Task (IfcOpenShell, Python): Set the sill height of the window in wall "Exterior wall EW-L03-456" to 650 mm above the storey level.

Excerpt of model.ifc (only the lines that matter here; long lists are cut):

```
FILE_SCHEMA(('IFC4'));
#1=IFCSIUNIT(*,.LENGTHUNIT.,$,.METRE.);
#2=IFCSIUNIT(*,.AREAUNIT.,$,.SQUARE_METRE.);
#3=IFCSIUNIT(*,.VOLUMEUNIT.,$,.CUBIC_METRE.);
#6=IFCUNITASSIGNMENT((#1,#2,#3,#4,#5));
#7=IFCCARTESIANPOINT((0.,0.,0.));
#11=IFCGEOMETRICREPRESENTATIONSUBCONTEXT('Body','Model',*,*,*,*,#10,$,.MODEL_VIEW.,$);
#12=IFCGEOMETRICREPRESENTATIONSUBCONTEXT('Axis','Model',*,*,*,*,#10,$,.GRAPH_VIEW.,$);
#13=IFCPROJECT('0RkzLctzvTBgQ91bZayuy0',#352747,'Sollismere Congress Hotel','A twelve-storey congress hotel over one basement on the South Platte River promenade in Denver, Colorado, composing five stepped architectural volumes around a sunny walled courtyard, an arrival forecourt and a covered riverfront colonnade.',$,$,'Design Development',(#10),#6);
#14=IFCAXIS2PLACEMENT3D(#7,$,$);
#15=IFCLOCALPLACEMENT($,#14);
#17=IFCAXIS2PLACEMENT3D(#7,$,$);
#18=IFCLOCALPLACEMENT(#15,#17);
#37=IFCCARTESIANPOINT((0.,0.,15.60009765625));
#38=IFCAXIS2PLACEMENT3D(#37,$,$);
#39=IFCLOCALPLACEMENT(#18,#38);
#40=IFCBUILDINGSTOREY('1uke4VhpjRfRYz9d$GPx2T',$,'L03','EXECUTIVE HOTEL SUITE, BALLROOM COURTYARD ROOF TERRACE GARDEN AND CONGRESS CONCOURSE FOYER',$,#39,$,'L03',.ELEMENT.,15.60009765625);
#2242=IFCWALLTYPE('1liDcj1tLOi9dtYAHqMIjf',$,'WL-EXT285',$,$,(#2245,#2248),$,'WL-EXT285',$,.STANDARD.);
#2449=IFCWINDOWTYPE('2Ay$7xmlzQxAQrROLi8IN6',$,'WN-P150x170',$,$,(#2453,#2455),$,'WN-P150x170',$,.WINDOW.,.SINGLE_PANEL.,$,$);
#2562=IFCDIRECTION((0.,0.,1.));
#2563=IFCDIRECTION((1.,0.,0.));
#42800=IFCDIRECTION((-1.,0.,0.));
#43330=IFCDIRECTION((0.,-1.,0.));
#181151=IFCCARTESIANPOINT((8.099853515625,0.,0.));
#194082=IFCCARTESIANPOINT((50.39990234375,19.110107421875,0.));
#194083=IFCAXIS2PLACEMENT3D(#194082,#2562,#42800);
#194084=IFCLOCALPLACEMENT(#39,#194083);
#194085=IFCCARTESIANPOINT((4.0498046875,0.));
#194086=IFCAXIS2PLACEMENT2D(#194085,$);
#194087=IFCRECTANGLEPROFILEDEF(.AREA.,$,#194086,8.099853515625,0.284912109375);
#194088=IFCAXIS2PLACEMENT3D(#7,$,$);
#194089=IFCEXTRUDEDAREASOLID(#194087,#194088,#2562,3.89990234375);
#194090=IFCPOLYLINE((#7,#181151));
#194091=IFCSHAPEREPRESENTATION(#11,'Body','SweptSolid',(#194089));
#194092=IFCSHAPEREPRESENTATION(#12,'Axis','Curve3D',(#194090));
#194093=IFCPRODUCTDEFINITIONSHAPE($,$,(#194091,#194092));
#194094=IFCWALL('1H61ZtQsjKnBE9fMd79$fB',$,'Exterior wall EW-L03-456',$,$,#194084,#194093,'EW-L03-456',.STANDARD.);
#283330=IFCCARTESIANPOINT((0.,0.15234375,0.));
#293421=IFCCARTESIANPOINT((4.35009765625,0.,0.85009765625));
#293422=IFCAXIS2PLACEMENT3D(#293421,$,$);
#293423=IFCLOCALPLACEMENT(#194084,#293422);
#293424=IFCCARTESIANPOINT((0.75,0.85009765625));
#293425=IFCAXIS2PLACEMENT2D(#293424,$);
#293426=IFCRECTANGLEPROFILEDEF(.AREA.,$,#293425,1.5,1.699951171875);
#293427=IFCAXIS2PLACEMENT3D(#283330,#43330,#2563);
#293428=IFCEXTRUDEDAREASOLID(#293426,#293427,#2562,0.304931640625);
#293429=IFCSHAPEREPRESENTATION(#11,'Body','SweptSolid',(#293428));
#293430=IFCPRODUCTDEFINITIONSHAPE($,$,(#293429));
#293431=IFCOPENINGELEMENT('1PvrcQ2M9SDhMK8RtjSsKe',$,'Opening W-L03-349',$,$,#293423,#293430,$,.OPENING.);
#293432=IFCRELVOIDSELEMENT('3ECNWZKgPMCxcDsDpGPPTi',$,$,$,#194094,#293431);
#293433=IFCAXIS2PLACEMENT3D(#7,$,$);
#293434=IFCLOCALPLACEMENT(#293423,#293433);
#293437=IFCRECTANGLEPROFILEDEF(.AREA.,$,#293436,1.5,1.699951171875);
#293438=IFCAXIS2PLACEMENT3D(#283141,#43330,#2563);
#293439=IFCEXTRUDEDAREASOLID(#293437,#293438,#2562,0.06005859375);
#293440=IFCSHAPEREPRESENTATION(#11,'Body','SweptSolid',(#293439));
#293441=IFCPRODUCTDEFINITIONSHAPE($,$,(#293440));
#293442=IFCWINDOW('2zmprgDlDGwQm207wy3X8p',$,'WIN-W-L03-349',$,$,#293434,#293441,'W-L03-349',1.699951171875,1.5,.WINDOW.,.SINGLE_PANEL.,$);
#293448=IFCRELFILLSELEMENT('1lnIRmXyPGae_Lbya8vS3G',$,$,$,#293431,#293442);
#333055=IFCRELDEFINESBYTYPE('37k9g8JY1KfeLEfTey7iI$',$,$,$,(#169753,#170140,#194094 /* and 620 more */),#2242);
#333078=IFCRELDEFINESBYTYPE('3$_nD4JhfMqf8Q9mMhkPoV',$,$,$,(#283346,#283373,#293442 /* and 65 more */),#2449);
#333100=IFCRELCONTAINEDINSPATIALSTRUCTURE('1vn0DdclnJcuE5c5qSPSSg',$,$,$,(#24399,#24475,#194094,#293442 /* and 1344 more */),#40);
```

```python
import numpy as np
import ifcopenshell
import ifcopenshell.api.geometry
import ifcopenshell.geom
import ifcopenshell.util.element
import ifcopenshell.util.placement
import ifcopenshell.util.shape
import ifcopenshell.util.unit

model = ifcopenshell.open("model.ifc")
unit_scale = ifcopenshell.util.unit.calculate_unit_scale(model)

window = model.by_guid("2zmprgDlDGwQm207wy3X8p")
opening = window.FillsVoids[0].RelatingOpeningElement
storey = ifcopenshell.util.element.get_container(window, ifc_class="IfcBuildingStorey")
level = ifcopenshell.util.placement.get_local_placement(storey.ObjectPlacement)[2, 3]

# The opening's origin need not be at the sill, so measure its lowest point.
shape = ifcopenshell.geom.create_shape(ifcopenshell.geom.settings(), opening)
bottom = ifcopenshell.util.shape.get_shape_bottom_elevation(shape, shape.geometry) / unit_scale
dz = level + 0.65 / unit_scale - bottom

shift = np.array([0.0, 0.0, dz])
# The window is placed relative to its opening, so it follows when the opening moves.
matrix = ifcopenshell.util.placement.get_local_placement(opening.ObjectPlacement)
matrix[:3, 3] += shift
ifcopenshell.api.geometry.edit_object_placement(
    model, product=opening, matrix=matrix, is_si=False, should_transform_children=True
)

print(f"moved by {dz * unit_scale:+.3f} m")

model.write("model_rev.ifc")
```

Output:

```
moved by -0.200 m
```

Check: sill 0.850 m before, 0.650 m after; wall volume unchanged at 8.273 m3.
